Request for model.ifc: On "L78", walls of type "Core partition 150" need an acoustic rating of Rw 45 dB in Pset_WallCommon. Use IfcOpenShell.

First a look at what the model holds.

```python
import ifcopenshell
import ifcopenshell.util.element

model = ifcopenshell.open("model.ifc")
print(model.schema)
storey = next(s for s in model.by_type("IfcBuildingStorey") if s.Name == "L78")
walls = [e for e in ifcopenshell.util.element.get_decomposition(storey) if e.is_a("IfcWall")]
seen = {}
for e in walls:
    element_type = ifcopenshell.util.element.get_type(e)
    key = (element_type.Name if element_type != e and element_type else None, ifcopenshell.util.element.get_pset(e, "Pset_WallCommon", "AcousticRating"))
    seen[key] = seen.get(key, 0) + 1
for (name, value), count in sorted(seen.items(), key=str):
    print(count, "x", name, "|", value)
```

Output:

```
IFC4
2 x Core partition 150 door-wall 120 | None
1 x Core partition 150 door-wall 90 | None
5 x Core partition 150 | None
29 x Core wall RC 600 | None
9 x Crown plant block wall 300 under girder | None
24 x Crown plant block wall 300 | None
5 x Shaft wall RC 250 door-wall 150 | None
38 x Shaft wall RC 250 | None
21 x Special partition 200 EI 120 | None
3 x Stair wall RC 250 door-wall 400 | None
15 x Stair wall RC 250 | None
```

```python
import ifcopenshell
import ifcopenshell.api.pset
import ifcopenshell.util.element

model = ifcopenshell.open("model.ifc")

storey = next(s for s in model.by_type("IfcBuildingStorey") if s.Name == "L78")
walls = [e for e in ifcopenshell.util.element.get_decomposition(storey) if e.is_a("IfcWall")]

count = 0
for e in walls:
    element_type = ifcopenshell.util.element.get_type(e)
    if element_type in (None, e) or element_type.Name != "Core partition 150":
        continue
    found = ifcopenshell.util.element.get_pset(e, "Pset_WallCommon", should_inherit=False)
    if found:
        pset = model.by_id(found["id"])
        if len(ifcopenshell.util.element.get_elements_by_pset(pset)) > 1:
            pset = ifcopenshell.api.pset.unshare_pset(model, products=[e], pset=pset)[0]
    else:
        pset = ifcopenshell.api.pset.add_pset(model, product=e, name="Pset_WallCommon")
    ifcopenshell.api.pset.edit_pset(model, pset=pset, properties={"AcousticRating": "Rw 45 dB"})
    count += 1

print(count, "walls updated")

model.write("model_rev.ifc")
```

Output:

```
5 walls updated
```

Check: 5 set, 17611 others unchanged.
